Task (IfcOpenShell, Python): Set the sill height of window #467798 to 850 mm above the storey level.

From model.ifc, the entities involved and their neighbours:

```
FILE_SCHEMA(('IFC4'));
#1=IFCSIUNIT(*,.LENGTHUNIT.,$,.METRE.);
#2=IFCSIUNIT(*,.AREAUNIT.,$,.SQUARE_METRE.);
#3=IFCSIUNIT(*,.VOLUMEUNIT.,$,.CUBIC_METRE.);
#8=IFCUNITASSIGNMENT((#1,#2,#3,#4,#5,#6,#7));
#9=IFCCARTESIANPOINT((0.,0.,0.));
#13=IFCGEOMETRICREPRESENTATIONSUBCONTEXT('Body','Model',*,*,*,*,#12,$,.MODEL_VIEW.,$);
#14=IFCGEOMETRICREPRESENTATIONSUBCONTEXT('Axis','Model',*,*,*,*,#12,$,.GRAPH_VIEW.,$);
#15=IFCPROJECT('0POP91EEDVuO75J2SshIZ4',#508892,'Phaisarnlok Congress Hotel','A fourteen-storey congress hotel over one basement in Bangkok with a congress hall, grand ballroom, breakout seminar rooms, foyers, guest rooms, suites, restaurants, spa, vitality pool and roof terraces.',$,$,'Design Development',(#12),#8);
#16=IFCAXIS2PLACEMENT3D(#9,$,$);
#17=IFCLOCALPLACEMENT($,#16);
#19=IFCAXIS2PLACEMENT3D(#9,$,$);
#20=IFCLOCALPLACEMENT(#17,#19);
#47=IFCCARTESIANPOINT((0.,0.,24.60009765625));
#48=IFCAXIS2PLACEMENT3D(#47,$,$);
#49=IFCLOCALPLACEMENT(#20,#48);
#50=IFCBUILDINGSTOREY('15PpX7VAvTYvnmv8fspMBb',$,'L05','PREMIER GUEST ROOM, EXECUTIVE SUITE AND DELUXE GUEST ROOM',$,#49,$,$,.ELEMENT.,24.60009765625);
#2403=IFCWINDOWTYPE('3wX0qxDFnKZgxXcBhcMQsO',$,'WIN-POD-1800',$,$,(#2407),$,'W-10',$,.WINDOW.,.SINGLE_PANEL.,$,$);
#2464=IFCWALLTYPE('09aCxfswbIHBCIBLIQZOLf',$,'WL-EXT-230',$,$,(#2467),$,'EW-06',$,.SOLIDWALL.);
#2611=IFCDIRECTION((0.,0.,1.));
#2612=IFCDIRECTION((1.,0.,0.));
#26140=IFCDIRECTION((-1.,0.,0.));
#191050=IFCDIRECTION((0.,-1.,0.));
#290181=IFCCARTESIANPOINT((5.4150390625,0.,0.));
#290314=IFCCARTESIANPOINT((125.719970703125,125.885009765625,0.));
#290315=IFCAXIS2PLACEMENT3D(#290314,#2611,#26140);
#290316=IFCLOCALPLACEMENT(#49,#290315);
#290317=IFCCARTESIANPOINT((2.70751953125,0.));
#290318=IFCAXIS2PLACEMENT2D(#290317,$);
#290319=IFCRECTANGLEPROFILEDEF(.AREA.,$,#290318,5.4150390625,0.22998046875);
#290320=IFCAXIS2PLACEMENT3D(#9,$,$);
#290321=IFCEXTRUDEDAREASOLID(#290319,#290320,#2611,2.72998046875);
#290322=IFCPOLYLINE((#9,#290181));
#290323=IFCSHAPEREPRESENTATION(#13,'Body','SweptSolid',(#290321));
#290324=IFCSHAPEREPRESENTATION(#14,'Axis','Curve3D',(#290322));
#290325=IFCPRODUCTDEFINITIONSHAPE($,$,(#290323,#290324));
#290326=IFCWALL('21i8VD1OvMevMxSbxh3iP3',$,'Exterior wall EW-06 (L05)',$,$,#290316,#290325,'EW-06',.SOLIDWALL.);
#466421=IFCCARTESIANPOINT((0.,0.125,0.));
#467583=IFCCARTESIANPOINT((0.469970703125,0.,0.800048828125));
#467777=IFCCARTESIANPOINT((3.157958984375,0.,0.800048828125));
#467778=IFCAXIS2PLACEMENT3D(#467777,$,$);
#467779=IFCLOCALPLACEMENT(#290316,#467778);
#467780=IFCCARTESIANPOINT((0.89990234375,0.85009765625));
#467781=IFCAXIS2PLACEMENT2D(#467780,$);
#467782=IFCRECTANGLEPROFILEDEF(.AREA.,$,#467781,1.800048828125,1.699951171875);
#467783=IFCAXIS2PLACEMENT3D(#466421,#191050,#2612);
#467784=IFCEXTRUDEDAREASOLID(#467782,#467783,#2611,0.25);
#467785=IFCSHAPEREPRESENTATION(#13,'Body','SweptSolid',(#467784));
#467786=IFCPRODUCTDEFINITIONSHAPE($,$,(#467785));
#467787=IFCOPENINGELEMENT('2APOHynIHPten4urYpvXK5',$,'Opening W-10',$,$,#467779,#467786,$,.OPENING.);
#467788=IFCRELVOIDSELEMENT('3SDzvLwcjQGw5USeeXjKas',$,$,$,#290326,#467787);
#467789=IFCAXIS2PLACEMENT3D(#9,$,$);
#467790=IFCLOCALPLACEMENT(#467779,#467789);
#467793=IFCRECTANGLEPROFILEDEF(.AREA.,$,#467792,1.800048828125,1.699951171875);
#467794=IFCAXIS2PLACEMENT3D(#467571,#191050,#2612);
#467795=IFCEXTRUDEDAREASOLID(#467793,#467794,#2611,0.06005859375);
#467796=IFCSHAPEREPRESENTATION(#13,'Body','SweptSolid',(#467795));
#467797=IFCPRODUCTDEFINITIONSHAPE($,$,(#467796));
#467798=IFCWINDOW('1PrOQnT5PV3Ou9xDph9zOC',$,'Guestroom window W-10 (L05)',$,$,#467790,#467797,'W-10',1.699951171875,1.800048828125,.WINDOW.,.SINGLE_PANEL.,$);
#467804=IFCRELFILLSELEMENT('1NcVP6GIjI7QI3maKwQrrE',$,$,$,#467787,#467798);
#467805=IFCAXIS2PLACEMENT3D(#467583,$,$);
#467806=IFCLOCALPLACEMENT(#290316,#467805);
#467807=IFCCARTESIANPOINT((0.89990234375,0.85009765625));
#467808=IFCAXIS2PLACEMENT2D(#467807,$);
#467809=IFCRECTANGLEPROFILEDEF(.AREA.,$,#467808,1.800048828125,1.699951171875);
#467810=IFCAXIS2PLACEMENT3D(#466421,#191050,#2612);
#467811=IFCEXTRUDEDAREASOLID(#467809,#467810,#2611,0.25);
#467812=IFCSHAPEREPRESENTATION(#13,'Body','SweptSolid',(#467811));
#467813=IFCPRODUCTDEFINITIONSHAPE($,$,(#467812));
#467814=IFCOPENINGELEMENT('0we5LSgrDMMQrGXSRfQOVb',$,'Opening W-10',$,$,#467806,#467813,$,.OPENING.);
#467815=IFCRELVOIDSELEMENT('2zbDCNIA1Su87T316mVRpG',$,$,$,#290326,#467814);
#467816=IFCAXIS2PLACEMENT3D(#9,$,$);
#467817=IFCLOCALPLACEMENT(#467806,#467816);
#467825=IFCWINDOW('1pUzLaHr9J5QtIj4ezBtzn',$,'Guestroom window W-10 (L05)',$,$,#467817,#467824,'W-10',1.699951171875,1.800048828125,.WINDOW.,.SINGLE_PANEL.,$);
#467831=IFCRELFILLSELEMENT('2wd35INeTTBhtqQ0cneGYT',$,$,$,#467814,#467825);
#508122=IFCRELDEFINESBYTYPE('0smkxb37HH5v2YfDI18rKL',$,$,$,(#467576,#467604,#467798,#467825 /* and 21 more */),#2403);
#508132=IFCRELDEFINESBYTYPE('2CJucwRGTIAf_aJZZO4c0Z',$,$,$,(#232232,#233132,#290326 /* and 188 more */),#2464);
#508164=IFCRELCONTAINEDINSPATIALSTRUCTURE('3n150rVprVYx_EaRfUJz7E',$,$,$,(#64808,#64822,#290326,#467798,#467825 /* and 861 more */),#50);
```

```python
import numpy as np
import ifcopenshell
import ifcopenshell.api.geometry
import ifcopenshell.geom
import ifcopenshell.util.element
import ifcopenshell.util.placement
import ifcopenshell.util.shape
import ifcopenshell.util.unit

model = ifcopenshell.open("model.ifc")
unit_scale = ifcopenshell.util.unit.calculate_unit_scale(model)

window = model.by_guid("1PrOQnT5PV3Ou9xDph9zOC")
opening = window.FillsVoids[0].RelatingOpeningElement
storey = ifcopenshell.util.element.get_container(window, ifc_class="IfcBuildingStorey")
level = ifcopenshell.util.placement.get_local_placement(storey.ObjectPlacement)[2, 3]

# The opening's origin need not be at the sill, so measure its lowest point.
shape = ifcopenshell.geom.create_shape(ifcopenshell.geom.settings(), opening)
bottom = ifcopenshell.util.shape.get_shape_bottom_elevation(shape, shape.geometry) / unit_scale
dz = level + 0.85 - bottom

shift = np.array([0.0, 0.0, dz])
# The window is placed relative to its opening, so it follows when the opening moves.
matrix = ifcopenshell.util.placement.get_local_placement(opening.ObjectPlacement)
matrix[:3, 3] += shift
ifcopenshell.api.geometry.edit_object_placement(
    model, product=opening, matrix=matrix, is_si=False, should_transform_children=True
)

print(f"moved by {dz * unit_scale:+.3f} m")

model.write("model_edited.ifc")
```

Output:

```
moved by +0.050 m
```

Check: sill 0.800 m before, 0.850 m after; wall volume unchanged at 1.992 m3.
